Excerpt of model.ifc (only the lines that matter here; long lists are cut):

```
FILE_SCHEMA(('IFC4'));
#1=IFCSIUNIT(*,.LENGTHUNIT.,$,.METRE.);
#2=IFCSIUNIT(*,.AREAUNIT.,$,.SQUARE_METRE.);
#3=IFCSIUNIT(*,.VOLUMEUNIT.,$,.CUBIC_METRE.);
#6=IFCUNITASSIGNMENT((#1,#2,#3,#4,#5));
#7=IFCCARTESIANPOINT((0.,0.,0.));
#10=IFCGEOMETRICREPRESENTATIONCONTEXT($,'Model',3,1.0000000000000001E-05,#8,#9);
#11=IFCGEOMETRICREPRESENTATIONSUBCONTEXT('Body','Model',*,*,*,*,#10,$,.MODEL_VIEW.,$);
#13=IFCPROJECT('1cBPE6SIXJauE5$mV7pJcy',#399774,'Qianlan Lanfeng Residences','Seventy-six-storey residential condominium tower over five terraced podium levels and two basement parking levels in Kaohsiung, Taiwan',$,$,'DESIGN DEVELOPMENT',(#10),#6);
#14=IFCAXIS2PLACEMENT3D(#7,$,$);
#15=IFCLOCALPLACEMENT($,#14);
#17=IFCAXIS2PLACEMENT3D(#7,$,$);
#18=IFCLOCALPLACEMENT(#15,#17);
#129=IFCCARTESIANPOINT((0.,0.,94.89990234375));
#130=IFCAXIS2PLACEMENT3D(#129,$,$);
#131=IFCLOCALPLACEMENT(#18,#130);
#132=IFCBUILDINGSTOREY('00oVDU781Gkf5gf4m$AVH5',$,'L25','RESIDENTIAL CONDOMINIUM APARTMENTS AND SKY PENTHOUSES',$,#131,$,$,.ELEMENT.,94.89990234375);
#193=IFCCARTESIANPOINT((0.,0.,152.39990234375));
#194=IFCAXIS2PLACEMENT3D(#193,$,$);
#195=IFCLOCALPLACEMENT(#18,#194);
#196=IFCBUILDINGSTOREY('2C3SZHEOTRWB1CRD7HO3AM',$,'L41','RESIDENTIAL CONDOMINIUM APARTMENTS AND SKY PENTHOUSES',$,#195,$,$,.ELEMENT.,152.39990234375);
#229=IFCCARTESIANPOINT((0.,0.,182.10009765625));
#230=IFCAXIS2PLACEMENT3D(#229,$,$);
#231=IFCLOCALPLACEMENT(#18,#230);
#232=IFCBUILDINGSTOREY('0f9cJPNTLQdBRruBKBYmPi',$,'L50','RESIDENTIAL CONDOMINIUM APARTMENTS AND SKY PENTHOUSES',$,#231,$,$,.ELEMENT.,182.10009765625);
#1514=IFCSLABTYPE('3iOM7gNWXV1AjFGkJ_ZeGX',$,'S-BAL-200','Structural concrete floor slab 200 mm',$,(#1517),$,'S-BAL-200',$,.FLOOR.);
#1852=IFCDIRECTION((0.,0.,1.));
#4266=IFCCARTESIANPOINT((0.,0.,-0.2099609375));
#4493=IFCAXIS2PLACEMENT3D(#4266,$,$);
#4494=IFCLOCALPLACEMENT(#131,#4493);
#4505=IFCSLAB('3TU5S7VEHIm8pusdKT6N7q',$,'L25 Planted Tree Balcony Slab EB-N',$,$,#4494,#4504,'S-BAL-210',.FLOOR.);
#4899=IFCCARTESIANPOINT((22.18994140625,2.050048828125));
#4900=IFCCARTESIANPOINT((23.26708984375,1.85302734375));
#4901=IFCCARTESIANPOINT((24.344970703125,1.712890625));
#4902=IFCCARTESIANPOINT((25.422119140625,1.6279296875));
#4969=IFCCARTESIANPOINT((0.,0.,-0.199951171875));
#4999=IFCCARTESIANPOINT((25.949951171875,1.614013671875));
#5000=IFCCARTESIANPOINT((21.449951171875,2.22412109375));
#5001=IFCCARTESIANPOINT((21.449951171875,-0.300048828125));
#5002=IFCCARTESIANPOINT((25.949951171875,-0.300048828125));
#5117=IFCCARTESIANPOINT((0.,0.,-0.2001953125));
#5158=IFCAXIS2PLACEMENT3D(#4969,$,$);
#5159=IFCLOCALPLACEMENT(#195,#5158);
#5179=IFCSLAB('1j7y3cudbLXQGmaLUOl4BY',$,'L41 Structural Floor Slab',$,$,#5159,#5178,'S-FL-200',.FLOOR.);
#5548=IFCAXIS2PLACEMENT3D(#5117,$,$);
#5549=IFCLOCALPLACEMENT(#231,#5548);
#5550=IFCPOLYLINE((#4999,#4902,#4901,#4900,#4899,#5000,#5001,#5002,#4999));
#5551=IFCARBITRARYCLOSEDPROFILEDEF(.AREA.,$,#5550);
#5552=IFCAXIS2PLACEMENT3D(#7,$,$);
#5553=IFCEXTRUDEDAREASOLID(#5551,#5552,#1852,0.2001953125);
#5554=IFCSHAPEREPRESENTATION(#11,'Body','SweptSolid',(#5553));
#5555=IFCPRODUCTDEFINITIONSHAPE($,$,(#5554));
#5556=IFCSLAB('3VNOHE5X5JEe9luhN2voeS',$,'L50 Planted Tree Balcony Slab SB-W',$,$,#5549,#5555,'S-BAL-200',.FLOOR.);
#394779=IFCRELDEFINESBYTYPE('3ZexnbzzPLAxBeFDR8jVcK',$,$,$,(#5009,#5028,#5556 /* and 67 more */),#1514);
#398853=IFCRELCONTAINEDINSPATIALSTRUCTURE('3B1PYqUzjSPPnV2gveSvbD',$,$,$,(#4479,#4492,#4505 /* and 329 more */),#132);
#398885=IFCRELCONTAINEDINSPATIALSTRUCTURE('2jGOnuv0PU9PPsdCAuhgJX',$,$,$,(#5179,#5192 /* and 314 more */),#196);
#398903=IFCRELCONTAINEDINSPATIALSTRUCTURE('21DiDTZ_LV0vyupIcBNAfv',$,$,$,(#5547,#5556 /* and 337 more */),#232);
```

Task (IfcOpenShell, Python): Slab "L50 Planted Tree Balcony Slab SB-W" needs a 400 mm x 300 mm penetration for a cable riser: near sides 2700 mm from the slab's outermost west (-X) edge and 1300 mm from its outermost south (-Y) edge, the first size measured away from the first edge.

```python
import numpy as np
import ifcopenshell
import ifcopenshell.api.feature
import ifcopenshell.api.geometry
import ifcopenshell.api.root
import ifcopenshell.geom
import ifcopenshell.util.placement
import ifcopenshell.util.representation
import ifcopenshell.util.shape
import ifcopenshell.util.unit

model = ifcopenshell.open("model.ifc")
unit_scale = ifcopenshell.util.unit.calculate_unit_scale(model)
settings = ifcopenshell.geom.settings()


def volume(element):
    """Net volume in cubic metres, openings subtracted."""
    shape = ifcopenshell.geom.create_shape(settings, element)
    return ifcopenshell.util.shape.get_volume(shape.geometry)


slab = model.by_guid("3VNOHE5X5JEe9luhN2voeS")
before = volume(slab)

# Extent in the slab's own axes, in metres. The edges named are its -X and -Y sides.
slab_shape = ifcopenshell.geom.create_shape(settings, slab)
vertices = ifcopenshell.util.shape.get_vertices(slab_shape.geometry)
x_min, y_min, bottom = vertices.min(axis=0)
top = vertices[:, 2].max()

opening = ifcopenshell.api.root.create_entity(model, ifc_class="IfcOpeningElement", name="Cable riser opening", predefined_type="OPENING")
context = ifcopenshell.util.representation.get_context(model, "Model", "Body", "MODEL_VIEW")
width, depth = 0.4, 0.3
outline = [(0.0, 0.0), (width, 0.0), (width, depth), (0.0, depth), (0.0, 0.0)]
# Overshoot both faces by 50 mm so the cut is clean.
shape = ifcopenshell.api.geometry.add_slab_representation(
    model, context=context, depth=top - bottom + 0.1, polyline=outline
)
ifcopenshell.api.geometry.assign_representation(model, product=opening, representation=shape)

matrix = ifcopenshell.util.placement.get_local_placement(slab.ObjectPlacement)
matrix[:, 3] = matrix @ np.append(np.array([x_min + 2.7, y_min + 1.3, bottom - 0.05]) / unit_scale, 1.0)
ifcopenshell.api.geometry.edit_object_placement(model, product=opening, matrix=matrix, is_si=False)
ifcopenshell.api.feature.add_feature(model, feature=opening, element=slab)

after = volume(slab)

print(f"slab volume {before:.3f} -> {after:.3f} m3")

model.write("model_rev.ifc")
```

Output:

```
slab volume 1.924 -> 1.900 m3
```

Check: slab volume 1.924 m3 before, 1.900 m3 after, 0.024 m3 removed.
